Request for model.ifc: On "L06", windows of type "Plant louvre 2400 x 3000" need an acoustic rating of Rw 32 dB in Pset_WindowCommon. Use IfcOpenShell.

First a look at what the model holds.

```python
import ifcopenshell
import ifcopenshell.util.element

model = ifcopenshell.open("model.ifc")
print(model.schema)
storey = next(s for s in model.by_type("IfcBuildingStorey") if s.Name == "L06")
windows = [e for e in ifcopenshell.util.element.get_decomposition(storey) if e.is_a("IfcWindow")]
seen = {}
for e in windows:
    element_type = ifcopenshell.util.element.get_type(e)
    key = (element_type.Name if element_type != e and element_type else None, ifcopenshell.util.element.get_pset(e, "Pset_WindowCommon", "AcousticRating"))
    seen[key] = seen.get(key, 0) + 1
for (name, value), count in sorted(seen.items(), key=str):
    print(count, "x", name, "|", value)
```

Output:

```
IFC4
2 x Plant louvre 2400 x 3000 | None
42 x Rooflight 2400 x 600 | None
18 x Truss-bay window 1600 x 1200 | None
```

```python
import ifcopenshell
import ifcopenshell.api.pset
import ifcopenshell.util.element

model = ifcopenshell.open("model.ifc")

storey = next(s for s in model.by_type("IfcBuildingStorey") if s.Name == "L06")
windows = [e for e in ifcopenshell.util.element.get_decomposition(storey) if e.is_a("IfcWindow")]

count = 0
for e in windows:
    element_type = ifcopenshell.util.element.get_type(e)
    if element_type in (None, e) or element_type.Name != "Plant louvre 2400 x 3000":
        continue
    # add_pset returns the element's existing set when there is one.
    pset = ifcopenshell.api.pset.add_pset(model, product=e, name="Pset_WindowCommon")
    ifcopenshell.api.pset.edit_pset(model, pset=pset, properties={"AcousticRating": "Rw 32 dB"})
    count += 1

print(count, "windows updated")

model.write("model_rev.ifc")
```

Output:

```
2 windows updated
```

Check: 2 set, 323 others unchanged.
